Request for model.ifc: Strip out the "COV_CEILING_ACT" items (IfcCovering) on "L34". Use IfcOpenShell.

First a look at what the model holds.

```python
import ifcopenshell
import ifcopenshell.util.element

model = ifcopenshell.open("model.ifc")
print(model.schema)
storey = next(s for s in model.by_type("IfcBuildingStorey") if s.Name == "L34")
coverings = [e for e in ifcopenshell.util.element.get_decomposition(storey) if e.is_a("IfcCovering")]
seen = {}
for e in coverings:
    element_type = ifcopenshell.util.element.get_type(e)
    name = element_type.Name if element_type not in (None, e) else None
    seen[name] = seen.get(name, 0) + 1
for name, count in sorted(seen.items(), key=str):
    print(count, "x", name)
```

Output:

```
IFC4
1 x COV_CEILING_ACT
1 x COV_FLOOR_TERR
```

```python
import ifcopenshell
import ifcopenshell.api.root
import ifcopenshell.util.element

model = ifcopenshell.open("model.ifc")

storey = next(s for s in model.by_type("IfcBuildingStorey") if s.Name == "L34")
coverings = [e for e in ifcopenshell.util.element.get_decomposition(storey) if e.is_a("IfcCovering")]
targets = [e for e in coverings if (t := ifcopenshell.util.element.get_type(e)) not in (None, e) and t.Name == "COV_CEILING_ACT"]

for e in targets:
    ifcopenshell.api.root.remove_product(model, product=e)
print(len(targets), "removed")

model.write("model_v2.ifc")
```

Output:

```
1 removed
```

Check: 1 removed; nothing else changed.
